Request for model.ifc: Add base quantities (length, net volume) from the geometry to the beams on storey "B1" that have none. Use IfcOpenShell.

First a look at what the model holds.

```python
import ifcopenshell
import ifcopenshell.util.element
import ifcopenshell.util.unit

model = ifcopenshell.open("model.ifc")
print(model.schema)
for unit_type in ("LENGTHUNIT", "AREAUNIT", "VOLUMEUNIT"):
    print(unit_type, ifcopenshell.util.unit.calculate_unit_scale(model, unit_type))
storey = next(s for s in model.by_type("IfcBuildingStorey") if s.Name == "B1")
beams = [e for e in ifcopenshell.util.element.get_decomposition(storey) if e.is_a("IfcBeam")]
for e in sorted(beams, key=lambda e: e.id()):
    print(e.id(), e.is_a(), e.Name, list(ifcopenshell.util.element.get_psets(e, qtos_only=True)), sep=" | ")
```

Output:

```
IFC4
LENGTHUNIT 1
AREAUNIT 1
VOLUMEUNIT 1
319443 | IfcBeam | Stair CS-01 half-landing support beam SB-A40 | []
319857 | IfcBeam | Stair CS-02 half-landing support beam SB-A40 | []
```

```python
import ifcopenshell
import ifcopenshell.api.pset
import ifcopenshell.geom
import ifcopenshell.util.element
import ifcopenshell.util.shape
import ifcopenshell.util.unit

model = ifcopenshell.open("model.ifc")
unit_scale = ifcopenshell.util.unit.calculate_unit_scale(model)
volume_scale = ifcopenshell.util.unit.calculate_unit_scale(model, "VOLUMEUNIT")
settings = ifcopenshell.geom.settings()

storey = next(s for s in model.by_type("IfcBuildingStorey") if s.Name == "B1")
beams = [e for e in ifcopenshell.util.element.get_decomposition(storey) if e.is_a("IfcBeam")]

for e in sorted(beams, key=lambda e: e.id()):
    if ifcopenshell.util.element.get_psets(e, qtos_only=True, should_inherit=False):
        continue
    # Geometry comes back in metres, in the element's own axes.
    shape = ifcopenshell.geom.create_shape(settings, e)
    values = {
        "Length": ifcopenshell.util.shape.get_max_xyz(shape.geometry) / unit_scale,
        "NetVolume": ifcopenshell.util.shape.get_volume(shape.geometry) / volume_scale,
    }
    qto = ifcopenshell.api.pset.add_qto(model, product=e, name="Qto_BeamBaseQuantities")
    ifcopenshell.api.pset.edit_qto(model, qto=qto, properties=values)
    print(e.id(), {k: round(v, 3) for k, v in values.items()})

model.write("model_v2.ifc")
```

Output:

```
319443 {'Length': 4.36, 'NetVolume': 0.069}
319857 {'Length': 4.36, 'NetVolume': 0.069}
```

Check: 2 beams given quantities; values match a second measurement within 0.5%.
